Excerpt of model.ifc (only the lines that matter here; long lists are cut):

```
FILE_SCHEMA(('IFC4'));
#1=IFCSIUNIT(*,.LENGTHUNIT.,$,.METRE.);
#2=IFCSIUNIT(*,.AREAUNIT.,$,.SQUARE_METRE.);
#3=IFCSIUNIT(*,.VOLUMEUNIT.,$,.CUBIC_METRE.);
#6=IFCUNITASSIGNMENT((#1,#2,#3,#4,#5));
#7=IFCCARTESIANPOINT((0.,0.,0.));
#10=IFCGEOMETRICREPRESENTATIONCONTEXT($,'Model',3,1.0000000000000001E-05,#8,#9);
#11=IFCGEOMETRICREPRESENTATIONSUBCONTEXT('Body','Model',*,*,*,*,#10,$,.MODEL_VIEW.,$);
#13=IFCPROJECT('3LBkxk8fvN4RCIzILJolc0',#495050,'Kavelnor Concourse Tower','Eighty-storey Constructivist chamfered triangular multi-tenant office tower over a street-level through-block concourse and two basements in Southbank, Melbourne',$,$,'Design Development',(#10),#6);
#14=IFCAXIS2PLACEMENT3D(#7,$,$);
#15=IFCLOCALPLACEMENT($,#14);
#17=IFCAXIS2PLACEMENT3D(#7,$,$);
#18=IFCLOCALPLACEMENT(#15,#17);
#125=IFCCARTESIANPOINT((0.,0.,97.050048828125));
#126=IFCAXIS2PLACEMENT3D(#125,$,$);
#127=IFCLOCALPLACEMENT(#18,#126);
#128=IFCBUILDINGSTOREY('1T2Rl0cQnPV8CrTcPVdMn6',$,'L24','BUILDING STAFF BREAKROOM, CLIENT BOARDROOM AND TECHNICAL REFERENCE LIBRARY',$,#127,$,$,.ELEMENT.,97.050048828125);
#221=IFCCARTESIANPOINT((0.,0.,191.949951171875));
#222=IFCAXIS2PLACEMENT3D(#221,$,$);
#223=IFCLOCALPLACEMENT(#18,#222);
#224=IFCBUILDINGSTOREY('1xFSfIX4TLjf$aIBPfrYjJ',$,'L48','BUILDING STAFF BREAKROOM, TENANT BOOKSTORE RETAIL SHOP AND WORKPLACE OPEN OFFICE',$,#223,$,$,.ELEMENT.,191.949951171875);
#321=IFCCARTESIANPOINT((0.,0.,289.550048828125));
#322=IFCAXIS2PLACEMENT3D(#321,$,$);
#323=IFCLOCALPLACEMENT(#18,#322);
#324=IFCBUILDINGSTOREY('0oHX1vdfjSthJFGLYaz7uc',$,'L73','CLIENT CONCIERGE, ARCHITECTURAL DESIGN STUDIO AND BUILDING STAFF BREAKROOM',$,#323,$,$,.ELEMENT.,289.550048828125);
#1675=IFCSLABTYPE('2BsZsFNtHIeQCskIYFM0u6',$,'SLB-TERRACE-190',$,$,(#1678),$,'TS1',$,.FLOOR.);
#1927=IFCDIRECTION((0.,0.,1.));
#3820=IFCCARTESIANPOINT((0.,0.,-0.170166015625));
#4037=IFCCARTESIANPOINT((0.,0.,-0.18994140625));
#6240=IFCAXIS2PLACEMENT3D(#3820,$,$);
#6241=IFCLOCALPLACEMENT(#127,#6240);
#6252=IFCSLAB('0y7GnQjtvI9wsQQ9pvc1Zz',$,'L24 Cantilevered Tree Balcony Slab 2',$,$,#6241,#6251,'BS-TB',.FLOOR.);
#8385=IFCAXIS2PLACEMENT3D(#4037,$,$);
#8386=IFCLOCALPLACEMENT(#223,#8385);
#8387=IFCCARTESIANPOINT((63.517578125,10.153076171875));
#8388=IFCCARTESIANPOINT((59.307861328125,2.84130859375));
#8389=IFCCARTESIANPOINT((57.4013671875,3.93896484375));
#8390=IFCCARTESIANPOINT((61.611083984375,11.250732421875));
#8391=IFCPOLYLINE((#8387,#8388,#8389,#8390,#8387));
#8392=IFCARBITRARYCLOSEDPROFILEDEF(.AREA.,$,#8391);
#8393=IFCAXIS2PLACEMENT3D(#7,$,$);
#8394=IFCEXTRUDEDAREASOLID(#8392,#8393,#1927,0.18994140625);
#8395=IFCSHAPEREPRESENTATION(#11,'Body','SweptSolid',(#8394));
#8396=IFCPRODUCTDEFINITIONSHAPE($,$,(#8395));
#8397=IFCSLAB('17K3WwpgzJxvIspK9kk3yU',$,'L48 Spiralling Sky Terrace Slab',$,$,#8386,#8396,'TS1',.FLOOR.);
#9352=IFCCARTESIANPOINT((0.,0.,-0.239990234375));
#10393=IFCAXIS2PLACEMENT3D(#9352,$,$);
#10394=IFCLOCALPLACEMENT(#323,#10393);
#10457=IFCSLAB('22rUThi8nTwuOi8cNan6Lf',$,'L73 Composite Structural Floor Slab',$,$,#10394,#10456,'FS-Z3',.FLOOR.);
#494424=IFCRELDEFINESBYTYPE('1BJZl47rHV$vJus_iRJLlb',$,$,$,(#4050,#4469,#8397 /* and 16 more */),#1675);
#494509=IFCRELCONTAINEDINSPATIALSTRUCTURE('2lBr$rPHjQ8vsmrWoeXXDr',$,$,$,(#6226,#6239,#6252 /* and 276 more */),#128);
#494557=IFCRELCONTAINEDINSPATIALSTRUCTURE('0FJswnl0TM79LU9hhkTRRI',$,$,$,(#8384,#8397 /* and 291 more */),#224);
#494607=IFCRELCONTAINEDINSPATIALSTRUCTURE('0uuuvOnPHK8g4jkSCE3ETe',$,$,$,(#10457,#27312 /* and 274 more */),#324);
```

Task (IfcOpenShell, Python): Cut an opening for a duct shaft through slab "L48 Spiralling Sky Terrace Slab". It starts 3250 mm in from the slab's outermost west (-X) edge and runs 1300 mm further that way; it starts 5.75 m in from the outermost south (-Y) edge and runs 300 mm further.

```python
import numpy as np
import ifcopenshell
import ifcopenshell.api.feature
import ifcopenshell.api.geometry
import ifcopenshell.api.root
import ifcopenshell.geom
import ifcopenshell.util.placement
import ifcopenshell.util.representation
import ifcopenshell.util.shape
import ifcopenshell.util.unit

model = ifcopenshell.open("model.ifc")
unit_scale = ifcopenshell.util.unit.calculate_unit_scale(model)
settings = ifcopenshell.geom.settings()


def volume(element):
    """Net volume in cubic metres, openings subtracted."""
    shape = ifcopenshell.geom.create_shape(settings, element)
    return ifcopenshell.util.shape.get_volume(shape.geometry)


slab = model.by_guid("17K3WwpgzJxvIspK9kk3yU")
before = volume(slab)

# Extent in the slab's own axes, in metres. The edges named are its -X and -Y sides.
slab_shape = ifcopenshell.geom.create_shape(settings, slab)
vertices = ifcopenshell.util.shape.get_vertices(slab_shape.geometry)
x_min, y_min, bottom = vertices.min(axis=0)
top = vertices[:, 2].max()

opening = ifcopenshell.api.root.create_entity(model, ifc_class="IfcOpeningElement", name="Duct shaft opening", predefined_type="OPENING")
context = ifcopenshell.util.representation.get_context(model, "Model", "Body", "MODEL_VIEW")
width, depth = 1.3, 0.3
outline = [(0.0, 0.0), (width, 0.0), (width, depth), (0.0, depth), (0.0, 0.0)]
# Overshoot both faces by 50 mm so the cut is clean.
shape = ifcopenshell.api.geometry.add_slab_representation(
    model, context=context, depth=top - bottom + 0.1, polyline=outline
)
ifcopenshell.api.geometry.assign_representation(model, product=opening, representation=shape)

matrix = ifcopenshell.util.placement.get_local_placement(slab.ObjectPlacement)
matrix[:, 3] = matrix @ np.append(np.array([x_min + 3.25, y_min + 5.75, bottom - 0.05]) / unit_scale, 1.0)
ifcopenshell.api.geometry.edit_object_placement(model, product=opening, matrix=matrix, is_si=False)
ifcopenshell.api.feature.add_feature(model, feature=opening, element=slab)

after = volume(slab)

print(f"slab volume {before:.3f} -> {after:.3f} m3")

model.write("model_updated.ifc")
```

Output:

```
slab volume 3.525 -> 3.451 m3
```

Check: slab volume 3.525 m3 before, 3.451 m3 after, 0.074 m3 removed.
